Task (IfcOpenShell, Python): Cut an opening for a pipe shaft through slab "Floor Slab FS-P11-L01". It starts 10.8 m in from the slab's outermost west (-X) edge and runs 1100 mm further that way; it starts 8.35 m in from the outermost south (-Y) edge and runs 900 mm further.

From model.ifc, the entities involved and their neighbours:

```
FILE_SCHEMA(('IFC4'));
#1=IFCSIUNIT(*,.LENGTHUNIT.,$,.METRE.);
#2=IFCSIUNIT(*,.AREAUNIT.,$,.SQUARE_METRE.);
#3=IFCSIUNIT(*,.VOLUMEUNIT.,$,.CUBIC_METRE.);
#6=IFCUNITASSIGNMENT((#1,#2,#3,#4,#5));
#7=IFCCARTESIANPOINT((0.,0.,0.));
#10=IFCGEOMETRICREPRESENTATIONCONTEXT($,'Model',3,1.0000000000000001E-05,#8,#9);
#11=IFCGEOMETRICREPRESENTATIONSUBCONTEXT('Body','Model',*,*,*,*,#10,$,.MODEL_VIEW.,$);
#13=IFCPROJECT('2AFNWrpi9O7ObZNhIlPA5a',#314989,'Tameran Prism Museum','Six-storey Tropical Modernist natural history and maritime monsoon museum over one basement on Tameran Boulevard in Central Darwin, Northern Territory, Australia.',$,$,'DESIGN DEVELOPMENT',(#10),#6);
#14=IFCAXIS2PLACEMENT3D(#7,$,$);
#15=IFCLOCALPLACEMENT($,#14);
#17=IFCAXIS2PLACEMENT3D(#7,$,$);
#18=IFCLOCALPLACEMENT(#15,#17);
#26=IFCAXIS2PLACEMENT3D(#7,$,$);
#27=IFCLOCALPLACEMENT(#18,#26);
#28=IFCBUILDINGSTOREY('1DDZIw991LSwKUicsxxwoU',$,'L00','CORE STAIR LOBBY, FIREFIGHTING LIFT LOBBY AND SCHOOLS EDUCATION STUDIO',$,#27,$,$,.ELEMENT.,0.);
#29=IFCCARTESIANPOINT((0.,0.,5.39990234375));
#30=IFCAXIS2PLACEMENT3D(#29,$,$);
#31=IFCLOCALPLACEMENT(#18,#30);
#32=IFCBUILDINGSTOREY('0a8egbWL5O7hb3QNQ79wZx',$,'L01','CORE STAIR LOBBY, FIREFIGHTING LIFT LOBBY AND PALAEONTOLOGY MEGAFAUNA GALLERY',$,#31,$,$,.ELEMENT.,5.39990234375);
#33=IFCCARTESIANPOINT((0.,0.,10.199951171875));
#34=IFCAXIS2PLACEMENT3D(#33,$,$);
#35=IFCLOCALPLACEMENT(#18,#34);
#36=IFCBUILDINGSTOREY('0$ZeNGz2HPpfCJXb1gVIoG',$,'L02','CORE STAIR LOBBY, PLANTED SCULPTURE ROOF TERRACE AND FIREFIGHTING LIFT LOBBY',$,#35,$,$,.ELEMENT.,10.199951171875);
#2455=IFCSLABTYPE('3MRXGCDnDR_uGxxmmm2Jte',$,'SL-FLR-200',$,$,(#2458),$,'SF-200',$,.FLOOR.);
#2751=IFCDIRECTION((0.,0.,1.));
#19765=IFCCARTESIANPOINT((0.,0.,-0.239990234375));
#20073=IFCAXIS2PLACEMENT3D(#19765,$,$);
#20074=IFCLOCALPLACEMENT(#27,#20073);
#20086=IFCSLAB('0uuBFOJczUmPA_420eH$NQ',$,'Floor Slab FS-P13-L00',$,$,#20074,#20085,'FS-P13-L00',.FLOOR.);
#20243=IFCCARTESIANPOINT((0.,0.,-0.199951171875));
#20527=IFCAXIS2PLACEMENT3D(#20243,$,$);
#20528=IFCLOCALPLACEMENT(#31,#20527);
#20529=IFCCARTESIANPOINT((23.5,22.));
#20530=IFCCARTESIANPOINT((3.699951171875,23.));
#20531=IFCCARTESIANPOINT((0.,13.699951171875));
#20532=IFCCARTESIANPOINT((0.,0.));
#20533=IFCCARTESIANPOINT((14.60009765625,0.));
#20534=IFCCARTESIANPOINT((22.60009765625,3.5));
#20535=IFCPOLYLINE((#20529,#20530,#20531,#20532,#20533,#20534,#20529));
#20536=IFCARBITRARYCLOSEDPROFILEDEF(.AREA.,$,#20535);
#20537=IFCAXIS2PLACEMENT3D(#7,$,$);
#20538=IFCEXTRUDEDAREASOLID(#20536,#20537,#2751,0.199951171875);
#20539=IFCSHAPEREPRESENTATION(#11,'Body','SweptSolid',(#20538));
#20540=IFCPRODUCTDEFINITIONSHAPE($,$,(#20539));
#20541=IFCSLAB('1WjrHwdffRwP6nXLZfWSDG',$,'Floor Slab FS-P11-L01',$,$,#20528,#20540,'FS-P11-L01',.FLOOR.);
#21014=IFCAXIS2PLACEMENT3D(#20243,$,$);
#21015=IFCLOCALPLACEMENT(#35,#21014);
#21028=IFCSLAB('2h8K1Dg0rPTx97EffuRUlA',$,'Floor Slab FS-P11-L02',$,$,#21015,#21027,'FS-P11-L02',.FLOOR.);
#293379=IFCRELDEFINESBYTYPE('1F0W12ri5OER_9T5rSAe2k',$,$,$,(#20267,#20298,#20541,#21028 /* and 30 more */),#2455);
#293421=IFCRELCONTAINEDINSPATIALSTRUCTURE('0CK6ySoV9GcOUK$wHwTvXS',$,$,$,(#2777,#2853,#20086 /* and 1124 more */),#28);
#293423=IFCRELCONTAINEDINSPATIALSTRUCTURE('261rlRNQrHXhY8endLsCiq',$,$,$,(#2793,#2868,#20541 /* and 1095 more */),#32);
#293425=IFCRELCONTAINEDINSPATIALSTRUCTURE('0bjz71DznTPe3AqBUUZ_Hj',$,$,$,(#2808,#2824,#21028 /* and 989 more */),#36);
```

```python
import numpy as np
import ifcopenshell
import ifcopenshell.api.feature
import ifcopenshell.api.geometry
import ifcopenshell.api.root
import ifcopenshell.geom
import ifcopenshell.util.placement
import ifcopenshell.util.representation
import ifcopenshell.util.shape
import ifcopenshell.util.unit

model = ifcopenshell.open("model.ifc")
unit_scale = ifcopenshell.util.unit.calculate_unit_scale(model)
settings = ifcopenshell.geom.settings()


def volume(element):
    """Net volume in cubic metres, openings subtracted."""
    shape = ifcopenshell.geom.create_shape(settings, element)
    return ifcopenshell.util.shape.get_volume(shape.geometry)


slab = model.by_guid("1WjrHwdffRwP6nXLZfWSDG")
before = volume(slab)

# Extent in the slab's own axes, in metres. The edges named are its -X and -Y sides.
slab_shape = ifcopenshell.geom.create_shape(settings, slab)
vertices = ifcopenshell.util.shape.get_vertices(slab_shape.geometry)
x_min, y_min, bottom = vertices.min(axis=0)
top = vertices[:, 2].max()

opening = ifcopenshell.api.root.create_entity(model, ifc_class="IfcOpeningElement", name="Pipe shaft opening", predefined_type="OPENING")
context = ifcopenshell.util.representation.get_context(model, "Model", "Body", "MODEL_VIEW")
width, depth = 1.1, 0.9
outline = [(0.0, 0.0), (width, 0.0), (width, depth), (0.0, depth), (0.0, 0.0)]
# Overshoot both faces by 50 mm so the cut is clean.
shape = ifcopenshell.api.geometry.add_slab_representation(
    model, context=context, depth=top - bottom + 0.1, polyline=outline
)
ifcopenshell.api.geometry.assign_representation(model, product=opening, representation=shape)

matrix = ifcopenshell.util.placement.get_local_placement(slab.ObjectPlacement)
matrix[:, 3] = matrix @ np.append(np.array([x_min + 10.8, y_min + 8.35, bottom - 0.05]) / unit_scale, 1.0)
ifcopenshell.api.geometry.edit_object_placement(model, product=opening, matrix=matrix, is_si=False)
ifcopenshell.api.feature.add_feature(model, feature=opening, element=slab)

after = volume(slab)

print(f"slab volume {before:.3f} -> {after:.3f} m3")

model.write("model_edited.ifc")
```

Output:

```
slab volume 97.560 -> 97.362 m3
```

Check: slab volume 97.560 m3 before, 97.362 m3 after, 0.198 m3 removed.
